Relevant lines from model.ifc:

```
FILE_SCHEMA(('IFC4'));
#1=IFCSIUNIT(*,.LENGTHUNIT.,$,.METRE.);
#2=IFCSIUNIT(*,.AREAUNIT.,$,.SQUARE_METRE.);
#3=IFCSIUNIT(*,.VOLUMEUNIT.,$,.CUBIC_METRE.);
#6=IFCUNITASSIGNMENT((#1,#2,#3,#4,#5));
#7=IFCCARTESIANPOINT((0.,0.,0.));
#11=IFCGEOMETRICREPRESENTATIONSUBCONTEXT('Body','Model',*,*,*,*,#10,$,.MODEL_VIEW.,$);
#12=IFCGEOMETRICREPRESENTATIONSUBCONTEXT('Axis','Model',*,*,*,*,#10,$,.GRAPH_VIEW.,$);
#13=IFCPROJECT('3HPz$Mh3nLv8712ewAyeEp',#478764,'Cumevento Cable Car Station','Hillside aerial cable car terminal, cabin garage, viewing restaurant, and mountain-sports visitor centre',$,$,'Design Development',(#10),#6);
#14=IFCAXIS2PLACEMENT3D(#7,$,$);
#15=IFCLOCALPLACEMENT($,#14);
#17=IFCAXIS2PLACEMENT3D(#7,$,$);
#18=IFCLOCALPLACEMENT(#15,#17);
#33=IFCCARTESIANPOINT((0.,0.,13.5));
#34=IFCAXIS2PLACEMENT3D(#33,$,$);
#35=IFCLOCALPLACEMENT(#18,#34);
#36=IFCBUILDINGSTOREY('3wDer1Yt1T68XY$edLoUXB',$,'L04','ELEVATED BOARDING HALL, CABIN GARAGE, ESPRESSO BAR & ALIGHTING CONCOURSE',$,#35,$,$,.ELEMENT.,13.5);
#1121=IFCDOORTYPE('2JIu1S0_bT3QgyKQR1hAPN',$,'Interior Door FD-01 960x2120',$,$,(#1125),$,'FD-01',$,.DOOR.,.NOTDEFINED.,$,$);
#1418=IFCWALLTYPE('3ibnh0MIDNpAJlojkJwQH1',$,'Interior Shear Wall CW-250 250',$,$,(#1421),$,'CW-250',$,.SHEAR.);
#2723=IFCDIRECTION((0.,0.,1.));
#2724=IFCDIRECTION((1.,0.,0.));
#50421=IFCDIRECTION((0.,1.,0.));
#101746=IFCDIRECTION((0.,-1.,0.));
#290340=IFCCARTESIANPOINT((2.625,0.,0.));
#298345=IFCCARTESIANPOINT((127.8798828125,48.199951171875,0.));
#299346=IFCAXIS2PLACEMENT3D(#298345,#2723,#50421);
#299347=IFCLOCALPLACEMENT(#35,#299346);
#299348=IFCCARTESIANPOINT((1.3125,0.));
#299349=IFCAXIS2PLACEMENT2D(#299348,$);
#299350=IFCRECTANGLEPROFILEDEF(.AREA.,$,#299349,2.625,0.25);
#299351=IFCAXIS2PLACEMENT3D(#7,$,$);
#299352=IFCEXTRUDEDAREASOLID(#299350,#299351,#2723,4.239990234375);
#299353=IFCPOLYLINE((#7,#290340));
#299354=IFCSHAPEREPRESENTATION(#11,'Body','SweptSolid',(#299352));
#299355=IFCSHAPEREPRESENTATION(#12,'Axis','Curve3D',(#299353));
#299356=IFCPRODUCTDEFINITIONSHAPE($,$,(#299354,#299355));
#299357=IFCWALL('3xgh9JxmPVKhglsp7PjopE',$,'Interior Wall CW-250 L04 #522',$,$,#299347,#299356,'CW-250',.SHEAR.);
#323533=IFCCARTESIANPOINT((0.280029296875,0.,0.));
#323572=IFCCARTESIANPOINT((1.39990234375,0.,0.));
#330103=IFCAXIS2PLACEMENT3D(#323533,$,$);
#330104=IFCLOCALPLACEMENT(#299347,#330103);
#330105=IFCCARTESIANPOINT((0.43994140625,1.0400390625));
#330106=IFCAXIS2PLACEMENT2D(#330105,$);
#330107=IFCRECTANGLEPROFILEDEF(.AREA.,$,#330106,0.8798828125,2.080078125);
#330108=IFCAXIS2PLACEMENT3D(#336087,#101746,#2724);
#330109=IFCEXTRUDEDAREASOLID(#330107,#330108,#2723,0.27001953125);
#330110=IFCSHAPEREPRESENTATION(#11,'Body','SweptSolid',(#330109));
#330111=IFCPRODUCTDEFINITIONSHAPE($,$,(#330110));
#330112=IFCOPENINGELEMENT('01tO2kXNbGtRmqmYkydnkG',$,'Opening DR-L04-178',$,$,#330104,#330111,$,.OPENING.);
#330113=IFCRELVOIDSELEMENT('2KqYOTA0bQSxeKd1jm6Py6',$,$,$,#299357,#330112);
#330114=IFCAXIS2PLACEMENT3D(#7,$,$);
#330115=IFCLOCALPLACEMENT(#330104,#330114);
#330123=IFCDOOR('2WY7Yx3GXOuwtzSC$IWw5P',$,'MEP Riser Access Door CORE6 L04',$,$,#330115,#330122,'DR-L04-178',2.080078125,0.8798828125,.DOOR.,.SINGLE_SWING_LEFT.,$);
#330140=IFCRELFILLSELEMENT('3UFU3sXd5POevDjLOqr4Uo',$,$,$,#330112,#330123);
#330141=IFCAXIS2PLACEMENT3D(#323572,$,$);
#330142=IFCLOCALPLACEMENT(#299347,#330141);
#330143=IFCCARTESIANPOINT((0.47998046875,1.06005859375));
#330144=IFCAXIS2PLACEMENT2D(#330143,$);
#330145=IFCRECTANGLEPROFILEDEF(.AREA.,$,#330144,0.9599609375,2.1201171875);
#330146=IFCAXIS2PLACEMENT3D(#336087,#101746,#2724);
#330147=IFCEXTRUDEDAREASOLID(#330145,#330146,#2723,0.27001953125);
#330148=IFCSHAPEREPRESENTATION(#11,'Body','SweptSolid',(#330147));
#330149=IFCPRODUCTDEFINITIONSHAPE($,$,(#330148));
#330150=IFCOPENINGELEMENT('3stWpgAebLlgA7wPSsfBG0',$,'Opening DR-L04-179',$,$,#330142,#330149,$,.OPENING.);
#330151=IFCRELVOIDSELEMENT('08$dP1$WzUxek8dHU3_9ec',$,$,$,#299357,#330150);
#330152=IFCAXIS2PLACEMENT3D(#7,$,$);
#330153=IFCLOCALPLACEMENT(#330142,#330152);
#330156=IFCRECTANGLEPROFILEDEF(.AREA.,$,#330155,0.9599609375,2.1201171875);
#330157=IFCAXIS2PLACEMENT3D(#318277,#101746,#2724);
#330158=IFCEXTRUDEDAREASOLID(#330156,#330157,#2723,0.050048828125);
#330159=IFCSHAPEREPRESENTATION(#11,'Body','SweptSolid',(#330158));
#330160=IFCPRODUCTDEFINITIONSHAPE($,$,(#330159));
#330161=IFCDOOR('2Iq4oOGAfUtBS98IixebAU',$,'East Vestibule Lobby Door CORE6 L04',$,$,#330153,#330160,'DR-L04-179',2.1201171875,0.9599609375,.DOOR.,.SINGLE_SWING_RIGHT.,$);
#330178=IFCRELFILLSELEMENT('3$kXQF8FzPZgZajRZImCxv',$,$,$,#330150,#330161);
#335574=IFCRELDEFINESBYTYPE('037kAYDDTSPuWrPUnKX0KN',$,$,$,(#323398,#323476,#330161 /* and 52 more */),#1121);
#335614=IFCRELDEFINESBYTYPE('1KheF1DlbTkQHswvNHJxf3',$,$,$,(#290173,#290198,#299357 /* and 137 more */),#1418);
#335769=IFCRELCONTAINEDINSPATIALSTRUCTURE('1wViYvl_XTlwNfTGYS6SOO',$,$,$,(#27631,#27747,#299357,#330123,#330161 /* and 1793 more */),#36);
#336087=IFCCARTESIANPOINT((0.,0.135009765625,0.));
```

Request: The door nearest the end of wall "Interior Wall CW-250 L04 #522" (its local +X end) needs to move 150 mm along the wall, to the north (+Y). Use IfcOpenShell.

```python
import ifcopenshell
import ifcopenshell.api.geometry
import ifcopenshell.util.placement
import ifcopenshell.util.unit

model = ifcopenshell.open("model.ifc")
unit_scale = ifcopenshell.util.unit.calculate_unit_scale(model)

door = model.by_guid("2Iq4oOGAfUtBS98IixebAU")
opening = door.FillsVoids[0].RelatingOpeningElement
wall = opening.VoidsElements[0].RelatingBuildingElement

wall_matrix = ifcopenshell.util.placement.get_local_placement(wall.ObjectPlacement)
shift = wall_matrix[:3, 0] * 0.15 / unit_scale
before = ifcopenshell.util.placement.get_local_placement(door.ObjectPlacement)[:3, 3].copy()

# The door is placed relative to its opening, so it follows when the opening moves.
matrix = ifcopenshell.util.placement.get_local_placement(opening.ObjectPlacement)
matrix[:3, 3] += shift
ifcopenshell.api.geometry.edit_object_placement(
    model, product=opening, matrix=matrix, is_si=False, should_transform_children=True
)

after = ifcopenshell.util.placement.get_local_placement(door.ObjectPlacement)[:3, 3]
print("door moved by", (after - before).round(3) + 0.0)

model.write("model-out.ifc")
```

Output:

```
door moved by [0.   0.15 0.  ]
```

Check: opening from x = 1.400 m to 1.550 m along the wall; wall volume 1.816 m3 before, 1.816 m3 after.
